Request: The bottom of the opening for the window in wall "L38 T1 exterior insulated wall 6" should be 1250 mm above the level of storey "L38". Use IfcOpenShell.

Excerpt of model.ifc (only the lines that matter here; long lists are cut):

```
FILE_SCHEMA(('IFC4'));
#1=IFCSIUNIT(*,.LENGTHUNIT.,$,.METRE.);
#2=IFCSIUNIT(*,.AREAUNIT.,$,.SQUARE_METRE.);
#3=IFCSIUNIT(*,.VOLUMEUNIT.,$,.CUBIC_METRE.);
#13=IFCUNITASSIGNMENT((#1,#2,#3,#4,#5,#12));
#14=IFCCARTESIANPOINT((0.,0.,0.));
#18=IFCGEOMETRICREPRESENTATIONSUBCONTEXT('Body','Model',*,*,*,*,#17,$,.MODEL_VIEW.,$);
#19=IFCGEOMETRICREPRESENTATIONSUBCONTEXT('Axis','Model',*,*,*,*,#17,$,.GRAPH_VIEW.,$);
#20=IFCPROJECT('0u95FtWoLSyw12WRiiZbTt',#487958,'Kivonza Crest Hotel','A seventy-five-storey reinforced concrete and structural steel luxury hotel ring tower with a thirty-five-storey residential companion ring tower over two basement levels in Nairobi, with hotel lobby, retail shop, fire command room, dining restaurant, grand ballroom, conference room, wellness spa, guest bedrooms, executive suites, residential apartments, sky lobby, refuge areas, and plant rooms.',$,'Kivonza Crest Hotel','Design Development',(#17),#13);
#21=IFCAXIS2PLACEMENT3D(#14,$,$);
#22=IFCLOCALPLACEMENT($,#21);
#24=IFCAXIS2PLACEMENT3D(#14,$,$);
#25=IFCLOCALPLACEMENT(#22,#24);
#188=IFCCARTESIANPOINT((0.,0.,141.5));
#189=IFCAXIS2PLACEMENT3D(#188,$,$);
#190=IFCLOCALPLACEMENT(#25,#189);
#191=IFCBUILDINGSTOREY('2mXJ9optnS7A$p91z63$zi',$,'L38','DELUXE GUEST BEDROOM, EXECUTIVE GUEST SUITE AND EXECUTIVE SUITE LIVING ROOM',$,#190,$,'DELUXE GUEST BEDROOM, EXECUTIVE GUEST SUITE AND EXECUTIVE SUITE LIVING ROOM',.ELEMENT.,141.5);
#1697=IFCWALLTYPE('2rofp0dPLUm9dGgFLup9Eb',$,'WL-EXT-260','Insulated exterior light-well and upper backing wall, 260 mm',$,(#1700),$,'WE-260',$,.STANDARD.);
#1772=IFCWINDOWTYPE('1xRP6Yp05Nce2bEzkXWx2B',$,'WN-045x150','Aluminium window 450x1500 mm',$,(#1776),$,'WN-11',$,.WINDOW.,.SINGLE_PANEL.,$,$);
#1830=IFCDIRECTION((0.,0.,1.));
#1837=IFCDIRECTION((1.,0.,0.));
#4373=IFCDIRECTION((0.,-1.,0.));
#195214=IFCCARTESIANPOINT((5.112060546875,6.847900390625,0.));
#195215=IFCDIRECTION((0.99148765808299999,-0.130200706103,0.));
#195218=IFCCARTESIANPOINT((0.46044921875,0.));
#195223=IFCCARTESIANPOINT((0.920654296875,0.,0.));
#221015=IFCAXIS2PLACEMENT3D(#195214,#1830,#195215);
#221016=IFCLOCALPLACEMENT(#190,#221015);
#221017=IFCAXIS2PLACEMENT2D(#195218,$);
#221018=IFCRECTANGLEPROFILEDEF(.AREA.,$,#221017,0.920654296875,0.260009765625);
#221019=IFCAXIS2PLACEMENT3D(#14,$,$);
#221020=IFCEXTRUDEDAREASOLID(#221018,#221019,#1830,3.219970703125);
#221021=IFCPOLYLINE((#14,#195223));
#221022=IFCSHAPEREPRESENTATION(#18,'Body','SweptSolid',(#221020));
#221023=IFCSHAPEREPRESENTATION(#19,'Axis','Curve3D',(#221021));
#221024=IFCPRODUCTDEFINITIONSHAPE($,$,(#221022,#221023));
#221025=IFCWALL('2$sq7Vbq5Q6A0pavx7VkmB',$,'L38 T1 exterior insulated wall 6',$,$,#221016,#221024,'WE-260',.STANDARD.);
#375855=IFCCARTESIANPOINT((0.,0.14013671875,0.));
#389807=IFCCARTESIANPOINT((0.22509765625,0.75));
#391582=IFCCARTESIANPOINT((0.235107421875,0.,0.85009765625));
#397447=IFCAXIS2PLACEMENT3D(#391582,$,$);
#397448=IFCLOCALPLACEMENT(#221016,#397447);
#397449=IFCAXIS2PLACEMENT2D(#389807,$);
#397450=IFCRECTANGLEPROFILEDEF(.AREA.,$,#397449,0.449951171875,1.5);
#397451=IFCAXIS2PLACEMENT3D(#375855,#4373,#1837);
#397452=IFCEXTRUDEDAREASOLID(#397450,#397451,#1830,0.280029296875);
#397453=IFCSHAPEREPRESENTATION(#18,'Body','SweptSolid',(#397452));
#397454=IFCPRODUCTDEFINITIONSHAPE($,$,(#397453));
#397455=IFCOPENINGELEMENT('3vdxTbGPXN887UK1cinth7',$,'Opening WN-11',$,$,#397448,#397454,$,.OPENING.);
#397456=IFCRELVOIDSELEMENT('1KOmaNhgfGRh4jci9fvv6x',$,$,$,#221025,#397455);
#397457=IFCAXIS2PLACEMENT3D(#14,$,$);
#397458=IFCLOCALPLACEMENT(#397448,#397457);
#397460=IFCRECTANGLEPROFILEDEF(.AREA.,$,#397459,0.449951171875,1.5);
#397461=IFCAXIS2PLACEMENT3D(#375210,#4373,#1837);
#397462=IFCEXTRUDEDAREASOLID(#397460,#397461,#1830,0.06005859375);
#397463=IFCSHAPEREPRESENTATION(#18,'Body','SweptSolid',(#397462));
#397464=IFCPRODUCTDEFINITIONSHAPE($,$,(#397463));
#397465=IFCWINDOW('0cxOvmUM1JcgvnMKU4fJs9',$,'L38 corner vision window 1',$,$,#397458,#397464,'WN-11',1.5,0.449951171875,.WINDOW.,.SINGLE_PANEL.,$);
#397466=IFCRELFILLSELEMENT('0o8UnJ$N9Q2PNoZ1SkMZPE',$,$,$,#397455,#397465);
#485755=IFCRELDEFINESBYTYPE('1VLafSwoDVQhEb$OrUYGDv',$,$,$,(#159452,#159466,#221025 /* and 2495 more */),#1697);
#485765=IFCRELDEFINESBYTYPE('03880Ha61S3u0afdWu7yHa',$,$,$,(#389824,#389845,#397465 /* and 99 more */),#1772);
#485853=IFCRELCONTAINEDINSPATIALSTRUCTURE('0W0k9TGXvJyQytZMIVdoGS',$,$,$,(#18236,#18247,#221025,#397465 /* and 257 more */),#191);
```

```python
import numpy as np
import ifcopenshell
import ifcopenshell.api.geometry
import ifcopenshell.geom
import ifcopenshell.util.element
import ifcopenshell.util.placement
import ifcopenshell.util.shape
import ifcopenshell.util.unit

model = ifcopenshell.open("model.ifc")
unit_scale = ifcopenshell.util.unit.calculate_unit_scale(model)

window = model.by_guid("0cxOvmUM1JcgvnMKU4fJs9")
opening = window.FillsVoids[0].RelatingOpeningElement
storey = ifcopenshell.util.element.get_container(window, ifc_class="IfcBuildingStorey")
level = ifcopenshell.util.placement.get_local_placement(storey.ObjectPlacement)[2, 3]

# The opening's origin need not be at the sill, so measure its lowest point.
shape = ifcopenshell.geom.create_shape(ifcopenshell.geom.settings(), opening)
bottom = ifcopenshell.util.shape.get_shape_bottom_elevation(shape, shape.geometry) / unit_scale
dz = level + 1.25 - bottom

shift = np.array([0.0, 0.0, dz])
# The window is placed relative to its opening, so it follows when the opening moves.
matrix = ifcopenshell.util.placement.get_local_placement(opening.ObjectPlacement)
matrix[:3, 3] += shift
ifcopenshell.api.geometry.edit_object_placement(
    model, product=opening, matrix=matrix, is_si=False, should_transform_children=True
)

print(f"moved by {dz * unit_scale:+.3f} m")

model.write("model-out.ifc")
```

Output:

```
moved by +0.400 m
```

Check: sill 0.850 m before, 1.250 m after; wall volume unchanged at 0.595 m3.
